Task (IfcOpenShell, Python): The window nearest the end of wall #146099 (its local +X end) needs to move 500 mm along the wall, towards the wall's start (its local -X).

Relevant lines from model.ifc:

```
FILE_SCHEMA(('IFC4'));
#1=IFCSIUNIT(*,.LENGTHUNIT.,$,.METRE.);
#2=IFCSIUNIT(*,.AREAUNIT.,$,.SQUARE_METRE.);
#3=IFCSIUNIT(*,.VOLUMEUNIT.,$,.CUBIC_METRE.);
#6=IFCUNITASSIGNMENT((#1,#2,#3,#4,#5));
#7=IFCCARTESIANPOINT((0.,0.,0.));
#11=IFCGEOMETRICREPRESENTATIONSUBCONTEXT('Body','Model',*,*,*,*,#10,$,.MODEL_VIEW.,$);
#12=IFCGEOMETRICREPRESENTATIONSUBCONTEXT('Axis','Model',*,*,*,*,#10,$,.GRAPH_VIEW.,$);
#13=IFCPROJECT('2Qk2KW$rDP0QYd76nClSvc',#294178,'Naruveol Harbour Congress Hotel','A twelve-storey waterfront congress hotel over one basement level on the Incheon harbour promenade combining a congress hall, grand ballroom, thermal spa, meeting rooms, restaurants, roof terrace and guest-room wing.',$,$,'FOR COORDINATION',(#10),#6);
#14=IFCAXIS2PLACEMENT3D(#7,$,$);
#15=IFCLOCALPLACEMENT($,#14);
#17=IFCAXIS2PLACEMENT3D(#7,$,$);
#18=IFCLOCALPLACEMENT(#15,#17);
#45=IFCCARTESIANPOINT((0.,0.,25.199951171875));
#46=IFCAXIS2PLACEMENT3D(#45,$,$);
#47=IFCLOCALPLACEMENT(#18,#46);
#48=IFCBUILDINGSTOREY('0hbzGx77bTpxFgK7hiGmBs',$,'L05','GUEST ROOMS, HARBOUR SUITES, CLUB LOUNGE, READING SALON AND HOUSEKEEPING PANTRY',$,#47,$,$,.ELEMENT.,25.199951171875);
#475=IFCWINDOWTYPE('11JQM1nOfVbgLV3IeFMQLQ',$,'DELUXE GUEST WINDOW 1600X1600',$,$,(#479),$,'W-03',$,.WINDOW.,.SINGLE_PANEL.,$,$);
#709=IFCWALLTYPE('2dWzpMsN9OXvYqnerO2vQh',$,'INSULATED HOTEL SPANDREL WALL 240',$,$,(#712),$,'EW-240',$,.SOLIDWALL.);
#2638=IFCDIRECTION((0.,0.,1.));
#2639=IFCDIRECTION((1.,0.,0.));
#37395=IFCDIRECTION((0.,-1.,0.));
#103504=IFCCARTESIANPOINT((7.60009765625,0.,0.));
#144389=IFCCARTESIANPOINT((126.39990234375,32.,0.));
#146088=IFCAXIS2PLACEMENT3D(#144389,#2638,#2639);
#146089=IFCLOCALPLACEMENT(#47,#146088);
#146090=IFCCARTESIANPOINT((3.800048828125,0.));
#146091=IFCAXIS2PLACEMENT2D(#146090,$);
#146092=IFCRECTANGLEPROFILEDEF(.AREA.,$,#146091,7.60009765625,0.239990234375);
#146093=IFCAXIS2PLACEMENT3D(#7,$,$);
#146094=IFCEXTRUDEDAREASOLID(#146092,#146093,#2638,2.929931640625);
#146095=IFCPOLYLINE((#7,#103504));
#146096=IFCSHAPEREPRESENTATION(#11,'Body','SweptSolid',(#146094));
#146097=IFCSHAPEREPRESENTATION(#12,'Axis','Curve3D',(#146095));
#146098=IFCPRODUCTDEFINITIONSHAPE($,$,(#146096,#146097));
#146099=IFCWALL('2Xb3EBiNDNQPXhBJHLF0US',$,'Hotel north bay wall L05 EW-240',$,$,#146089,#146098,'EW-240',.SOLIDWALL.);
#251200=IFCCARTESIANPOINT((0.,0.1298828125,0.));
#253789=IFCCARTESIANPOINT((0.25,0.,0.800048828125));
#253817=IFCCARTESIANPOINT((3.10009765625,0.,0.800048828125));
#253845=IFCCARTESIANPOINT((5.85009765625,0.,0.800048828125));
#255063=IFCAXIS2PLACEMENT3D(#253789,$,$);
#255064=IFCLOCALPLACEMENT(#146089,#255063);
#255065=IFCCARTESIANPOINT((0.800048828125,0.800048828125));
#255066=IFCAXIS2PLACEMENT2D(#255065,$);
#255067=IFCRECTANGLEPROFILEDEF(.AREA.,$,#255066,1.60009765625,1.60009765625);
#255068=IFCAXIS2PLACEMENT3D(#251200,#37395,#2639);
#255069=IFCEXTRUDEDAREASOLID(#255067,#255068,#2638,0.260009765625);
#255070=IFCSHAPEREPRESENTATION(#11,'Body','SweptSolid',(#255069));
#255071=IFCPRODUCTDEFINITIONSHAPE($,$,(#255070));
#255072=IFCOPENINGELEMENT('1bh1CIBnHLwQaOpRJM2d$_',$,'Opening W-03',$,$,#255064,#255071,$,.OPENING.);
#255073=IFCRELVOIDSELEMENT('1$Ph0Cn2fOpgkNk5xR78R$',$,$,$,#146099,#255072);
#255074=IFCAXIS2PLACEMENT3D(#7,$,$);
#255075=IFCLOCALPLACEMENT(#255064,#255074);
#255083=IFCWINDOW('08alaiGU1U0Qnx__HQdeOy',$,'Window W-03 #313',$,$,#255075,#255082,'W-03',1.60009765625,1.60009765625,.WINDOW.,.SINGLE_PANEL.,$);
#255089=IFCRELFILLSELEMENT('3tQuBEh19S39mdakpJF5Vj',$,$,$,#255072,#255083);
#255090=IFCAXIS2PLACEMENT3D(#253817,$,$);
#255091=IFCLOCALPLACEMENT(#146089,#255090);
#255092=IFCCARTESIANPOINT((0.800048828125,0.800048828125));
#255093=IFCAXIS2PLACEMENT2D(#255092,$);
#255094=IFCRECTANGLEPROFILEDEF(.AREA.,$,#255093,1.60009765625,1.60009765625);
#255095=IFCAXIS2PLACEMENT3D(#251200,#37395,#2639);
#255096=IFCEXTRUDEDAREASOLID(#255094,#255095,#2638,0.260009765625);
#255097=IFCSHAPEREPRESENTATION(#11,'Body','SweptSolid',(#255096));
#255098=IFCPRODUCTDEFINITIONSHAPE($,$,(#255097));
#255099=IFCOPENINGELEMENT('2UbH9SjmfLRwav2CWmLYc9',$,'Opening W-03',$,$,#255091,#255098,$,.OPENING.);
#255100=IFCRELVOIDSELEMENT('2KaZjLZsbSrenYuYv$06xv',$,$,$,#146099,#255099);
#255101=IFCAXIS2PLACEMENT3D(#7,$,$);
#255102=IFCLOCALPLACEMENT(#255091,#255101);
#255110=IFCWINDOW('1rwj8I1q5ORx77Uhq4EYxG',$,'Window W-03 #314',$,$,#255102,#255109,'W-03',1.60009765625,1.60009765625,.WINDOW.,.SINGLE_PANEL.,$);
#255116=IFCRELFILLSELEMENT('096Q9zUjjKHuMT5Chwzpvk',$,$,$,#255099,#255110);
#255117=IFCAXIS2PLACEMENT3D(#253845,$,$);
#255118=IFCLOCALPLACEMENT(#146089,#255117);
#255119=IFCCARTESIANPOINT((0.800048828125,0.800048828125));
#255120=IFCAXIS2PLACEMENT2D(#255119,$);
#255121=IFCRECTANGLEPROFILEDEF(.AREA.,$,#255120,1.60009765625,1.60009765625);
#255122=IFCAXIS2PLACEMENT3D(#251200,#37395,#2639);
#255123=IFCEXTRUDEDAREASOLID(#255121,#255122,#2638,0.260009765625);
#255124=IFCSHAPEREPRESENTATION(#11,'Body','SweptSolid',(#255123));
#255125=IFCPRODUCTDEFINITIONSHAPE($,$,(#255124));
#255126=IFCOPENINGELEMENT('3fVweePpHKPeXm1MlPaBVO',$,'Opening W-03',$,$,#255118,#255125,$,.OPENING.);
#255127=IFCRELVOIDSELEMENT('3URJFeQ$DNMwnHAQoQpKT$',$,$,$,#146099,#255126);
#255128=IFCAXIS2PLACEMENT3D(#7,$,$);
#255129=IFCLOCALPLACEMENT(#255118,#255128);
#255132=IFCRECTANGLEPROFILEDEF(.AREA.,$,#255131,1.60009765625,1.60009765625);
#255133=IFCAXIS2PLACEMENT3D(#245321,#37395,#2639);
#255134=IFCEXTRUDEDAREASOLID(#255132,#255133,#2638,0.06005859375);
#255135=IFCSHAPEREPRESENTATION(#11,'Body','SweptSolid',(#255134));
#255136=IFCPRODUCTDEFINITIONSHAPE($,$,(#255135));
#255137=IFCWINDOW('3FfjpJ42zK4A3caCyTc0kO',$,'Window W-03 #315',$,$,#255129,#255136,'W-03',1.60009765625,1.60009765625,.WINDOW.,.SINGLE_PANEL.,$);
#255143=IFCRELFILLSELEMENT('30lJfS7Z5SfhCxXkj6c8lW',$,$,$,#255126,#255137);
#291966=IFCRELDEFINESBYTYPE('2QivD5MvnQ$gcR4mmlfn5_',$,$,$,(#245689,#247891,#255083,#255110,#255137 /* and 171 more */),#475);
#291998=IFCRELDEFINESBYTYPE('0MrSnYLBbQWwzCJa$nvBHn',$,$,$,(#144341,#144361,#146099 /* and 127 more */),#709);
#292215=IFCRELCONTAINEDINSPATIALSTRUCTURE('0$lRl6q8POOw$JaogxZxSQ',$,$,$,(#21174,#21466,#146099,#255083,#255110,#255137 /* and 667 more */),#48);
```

```python
import ifcopenshell
import ifcopenshell.api.geometry
import ifcopenshell.util.placement

model = ifcopenshell.open("model.ifc")

window = model.by_guid("3FfjpJ42zK4A3caCyTc0kO")
opening = window.FillsVoids[0].RelatingOpeningElement
wall = opening.VoidsElements[0].RelatingBuildingElement

wall_matrix = ifcopenshell.util.placement.get_local_placement(wall.ObjectPlacement)
shift = wall_matrix[:3, 0] * -0.5
before = ifcopenshell.util.placement.get_local_placement(window.ObjectPlacement)[:3, 3].copy()

# The window is placed relative to its opening, so it follows when the opening moves.
matrix = ifcopenshell.util.placement.get_local_placement(opening.ObjectPlacement)
matrix[:3, 3] += shift
ifcopenshell.api.geometry.edit_object_placement(
    model, product=opening, matrix=matrix, is_si=False, should_transform_children=True
)

after = ifcopenshell.util.placement.get_local_placement(window.ObjectPlacement)[:3, 3]
print("window moved by", (after - before).round(3) + 0.0)

model.write("model_updated.ifc")
```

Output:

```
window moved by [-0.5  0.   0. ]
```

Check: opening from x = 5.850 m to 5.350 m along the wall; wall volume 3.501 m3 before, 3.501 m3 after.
